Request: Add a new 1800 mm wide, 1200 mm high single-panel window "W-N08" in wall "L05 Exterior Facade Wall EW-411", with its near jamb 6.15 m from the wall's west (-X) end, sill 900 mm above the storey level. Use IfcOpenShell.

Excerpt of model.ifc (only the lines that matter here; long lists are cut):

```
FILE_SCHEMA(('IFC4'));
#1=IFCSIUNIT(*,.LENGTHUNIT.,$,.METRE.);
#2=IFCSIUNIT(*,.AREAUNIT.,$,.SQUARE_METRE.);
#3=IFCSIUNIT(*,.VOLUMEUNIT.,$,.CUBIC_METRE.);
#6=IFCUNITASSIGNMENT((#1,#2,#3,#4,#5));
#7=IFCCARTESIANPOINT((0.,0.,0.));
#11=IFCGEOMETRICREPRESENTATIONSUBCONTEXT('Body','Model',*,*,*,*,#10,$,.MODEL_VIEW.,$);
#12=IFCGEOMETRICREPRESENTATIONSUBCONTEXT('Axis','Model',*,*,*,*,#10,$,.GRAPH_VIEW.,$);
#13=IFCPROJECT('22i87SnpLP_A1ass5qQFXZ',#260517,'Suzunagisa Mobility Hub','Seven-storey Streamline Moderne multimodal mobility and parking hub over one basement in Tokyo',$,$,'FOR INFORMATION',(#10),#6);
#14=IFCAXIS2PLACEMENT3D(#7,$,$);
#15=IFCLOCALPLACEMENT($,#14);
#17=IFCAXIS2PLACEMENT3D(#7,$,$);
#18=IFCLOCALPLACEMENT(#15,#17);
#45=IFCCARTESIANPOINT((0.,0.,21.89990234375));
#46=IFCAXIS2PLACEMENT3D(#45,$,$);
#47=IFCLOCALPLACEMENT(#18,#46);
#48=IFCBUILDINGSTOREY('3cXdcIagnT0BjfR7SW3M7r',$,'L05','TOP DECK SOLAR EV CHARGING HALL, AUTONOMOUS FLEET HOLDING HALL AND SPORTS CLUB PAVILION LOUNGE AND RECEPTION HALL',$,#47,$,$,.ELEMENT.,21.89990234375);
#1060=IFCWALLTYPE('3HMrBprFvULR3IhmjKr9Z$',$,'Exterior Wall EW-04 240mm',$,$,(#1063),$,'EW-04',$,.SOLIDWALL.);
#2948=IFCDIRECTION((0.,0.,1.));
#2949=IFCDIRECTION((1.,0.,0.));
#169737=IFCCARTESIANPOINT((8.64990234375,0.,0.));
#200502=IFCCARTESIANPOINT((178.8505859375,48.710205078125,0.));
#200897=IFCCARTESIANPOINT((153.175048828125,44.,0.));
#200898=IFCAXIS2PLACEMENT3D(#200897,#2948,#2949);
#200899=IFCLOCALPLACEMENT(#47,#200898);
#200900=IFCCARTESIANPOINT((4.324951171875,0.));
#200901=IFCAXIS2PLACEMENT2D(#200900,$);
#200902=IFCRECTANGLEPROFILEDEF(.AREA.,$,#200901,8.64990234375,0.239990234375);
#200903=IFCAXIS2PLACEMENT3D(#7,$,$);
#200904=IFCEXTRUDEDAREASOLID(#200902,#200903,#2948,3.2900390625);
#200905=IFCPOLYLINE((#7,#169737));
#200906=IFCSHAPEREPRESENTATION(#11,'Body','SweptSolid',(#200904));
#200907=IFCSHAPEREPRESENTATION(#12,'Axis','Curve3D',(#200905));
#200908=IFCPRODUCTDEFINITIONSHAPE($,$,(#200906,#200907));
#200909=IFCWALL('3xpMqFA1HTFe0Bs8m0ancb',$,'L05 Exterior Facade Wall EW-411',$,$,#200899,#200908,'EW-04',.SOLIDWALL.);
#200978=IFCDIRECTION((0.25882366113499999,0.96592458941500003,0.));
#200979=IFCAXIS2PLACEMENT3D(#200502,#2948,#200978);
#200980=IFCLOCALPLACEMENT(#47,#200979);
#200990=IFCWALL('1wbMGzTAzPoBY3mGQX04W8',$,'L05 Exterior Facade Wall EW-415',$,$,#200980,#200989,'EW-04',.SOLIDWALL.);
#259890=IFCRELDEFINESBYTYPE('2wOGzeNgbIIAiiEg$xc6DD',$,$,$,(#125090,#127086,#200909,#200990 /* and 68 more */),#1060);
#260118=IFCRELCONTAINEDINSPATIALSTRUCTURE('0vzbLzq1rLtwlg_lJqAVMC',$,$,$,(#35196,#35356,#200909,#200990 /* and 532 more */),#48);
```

```python
import numpy as np
import ifcopenshell
import ifcopenshell.api.feature
import ifcopenshell.api.geometry
import ifcopenshell.api.root
import ifcopenshell.api.spatial
import ifcopenshell.geom
import ifcopenshell.util.element
import ifcopenshell.util.placement
import ifcopenshell.util.representation
import ifcopenshell.util.shape
import ifcopenshell.util.unit

model = ifcopenshell.open("model.ifc")
unit_scale = ifcopenshell.util.unit.calculate_unit_scale(model)
settings = ifcopenshell.geom.settings()


def volume(element):
    """Net volume in cubic metres, openings subtracted."""
    shape = ifcopenshell.geom.create_shape(settings, element)
    return ifcopenshell.util.shape.get_volume(shape.geometry)


wall = model.by_id(200909)
storey = ifcopenshell.util.element.get_container(wall, ifc_class="IfcBuildingStorey")
context = ifcopenshell.util.representation.get_context(model, "Model", "Body", "MODEL_VIEW")
before = volume(wall)

width, height, from_end, sill = 1.8, 1.2, 6.15, 0.9  # metres

# The wall runs along its own X axis, and the end named is its -X end.
wall_shape = ifcopenshell.geom.create_shape(settings, wall)
x, y, z = ifcopenshell.util.shape.get_vertices(wall_shape.geometry).T
start = x.min() + from_end
face, thickness = float(y.min()), float(y.max() - y.min())
wall_matrix = ifcopenshell.util.placement.get_local_placement(wall.ObjectPlacement)
level = ifcopenshell.util.placement.get_local_placement(storey.ObjectPlacement)[2, 3]


def in_wall(x, y):
    """Placement at x, y metres in the wall's axes, at sill height."""
    matrix = wall_matrix.copy()
    matrix[:, 3] = wall_matrix @ np.array([x / unit_scale, y / unit_scale, 0.0, 1.0])
    matrix[2, 3] = level + sill / unit_scale
    return matrix


# Opening: a box that overshoots both wall faces by 50 mm.
opening = ifcopenshell.api.root.create_entity(model, ifc_class="IfcOpeningElement", predefined_type="OPENING")
box = ifcopenshell.api.geometry.add_wall_representation(
    model, context=context, length=width, height=height, thickness=thickness + 0.1
)
ifcopenshell.api.geometry.assign_representation(model, product=opening, representation=box)
ifcopenshell.api.geometry.edit_object_placement(model, product=opening, matrix=in_wall(start, face - 0.05), is_si=False)
ifcopenshell.api.feature.add_feature(model, feature=opening, element=wall)

window = ifcopenshell.api.root.create_entity(model, ifc_class="IfcWindow", name="W-N08", predefined_type="WINDOW")
window.OverallWidth, window.OverallHeight = width / unit_scale, height / unit_scale
window.PartitioningType = "SINGLE_PANEL"
body = ifcopenshell.api.geometry.add_window_representation(
    model,
    context=context,
    overall_width=window.OverallWidth,
    overall_height=window.OverallHeight,
    partition_type="SINGLE_PANEL",
)
ifcopenshell.api.geometry.assign_representation(model, product=window, representation=body)
ifcopenshell.api.spatial.assign_container(model, products=[window], relating_structure=storey)
ifcopenshell.api.feature.add_filling(model, opening=opening, element=window)

# Centre the window in the wall's thickness.
ifcopenshell.api.geometry.edit_object_placement(model, product=window, matrix=in_wall(start, face), is_si=False)
window_shape = ifcopenshell.geom.create_shape(settings, window)
depth = ifcopenshell.util.shape.get_vertices(window_shape.geometry)[:, 1]
offset = face + thickness / 2 - (depth.min() + depth.max()) / 2
ifcopenshell.api.geometry.edit_object_placement(model, product=window, matrix=in_wall(start, offset), is_si=False)

after = volume(wall)

print(f"wall volume {before:.3f} -> {after:.3f} m3")

model.write("model_edited.ifc")
```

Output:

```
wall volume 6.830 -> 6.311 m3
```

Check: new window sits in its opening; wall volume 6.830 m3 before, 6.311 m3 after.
